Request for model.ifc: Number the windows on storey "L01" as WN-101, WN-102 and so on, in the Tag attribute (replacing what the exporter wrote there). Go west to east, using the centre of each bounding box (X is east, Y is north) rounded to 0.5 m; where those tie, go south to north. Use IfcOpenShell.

First a look at what the model holds.

```python
import ifcopenshell
import ifcopenshell.util.element
import ifcopenshell.util.placement

model = ifcopenshell.open("model.ifc")
print(model.schema)
storey = next(s for s in model.by_type("IfcBuildingStorey") if s.Name == "L01")
windows = [e for e in ifcopenshell.util.element.get_decomposition(storey) if e.is_a("IfcWindow")]
for e in sorted(windows, key=lambda e: e.id()):
    origin = ifcopenshell.util.placement.get_local_placement(e.ObjectPlacement)[:3, 3]
    print(e.id(), e.Tag, e.Name, origin.round(2) + 0.0, sep=" | ")
```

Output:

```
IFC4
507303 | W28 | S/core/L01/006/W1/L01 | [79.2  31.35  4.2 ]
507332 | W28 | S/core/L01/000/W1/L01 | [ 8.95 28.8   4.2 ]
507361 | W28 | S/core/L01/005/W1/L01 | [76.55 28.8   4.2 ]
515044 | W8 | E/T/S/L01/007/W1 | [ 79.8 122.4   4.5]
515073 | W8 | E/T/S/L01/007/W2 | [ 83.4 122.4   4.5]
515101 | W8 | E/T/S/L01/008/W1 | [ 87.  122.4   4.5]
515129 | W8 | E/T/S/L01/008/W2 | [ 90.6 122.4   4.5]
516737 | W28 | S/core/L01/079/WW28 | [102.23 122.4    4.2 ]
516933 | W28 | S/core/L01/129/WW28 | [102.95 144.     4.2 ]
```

```python
import ifcopenshell
import ifcopenshell.geom
import ifcopenshell.util.element
import ifcopenshell.util.shape

model = ifcopenshell.open("model.ifc")
settings = ifcopenshell.geom.settings()
settings.set("use-world-coords", True)


def centre(element):
    shape = ifcopenshell.geom.create_shape(settings, element)
    return ifcopenshell.util.shape.get_bbox_centroid(shape.geometry)


storey = next(s for s in model.by_type("IfcBuildingStorey") if s.Name == "L01")
windows = [e for e in ifcopenshell.util.element.get_decomposition(storey) if e.is_a("IfcWindow")]

# Insertion points can sit at a corner or the storey origin, so sort by the geometry (in metres).
centres = {e: centre(e) for e in windows}
windows.sort(key=lambda e: (round(centres[e][0] / 0.5), centres[e][1]))

for i, e in enumerate(windows, start=1):
    number = f"WN-1{i:02d}"
    e.Tag = number
    print(e.id(), number)

model.write("model_rev.ifc")
```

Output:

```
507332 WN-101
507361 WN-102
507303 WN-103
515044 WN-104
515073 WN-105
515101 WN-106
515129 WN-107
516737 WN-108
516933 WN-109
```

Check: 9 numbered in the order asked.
